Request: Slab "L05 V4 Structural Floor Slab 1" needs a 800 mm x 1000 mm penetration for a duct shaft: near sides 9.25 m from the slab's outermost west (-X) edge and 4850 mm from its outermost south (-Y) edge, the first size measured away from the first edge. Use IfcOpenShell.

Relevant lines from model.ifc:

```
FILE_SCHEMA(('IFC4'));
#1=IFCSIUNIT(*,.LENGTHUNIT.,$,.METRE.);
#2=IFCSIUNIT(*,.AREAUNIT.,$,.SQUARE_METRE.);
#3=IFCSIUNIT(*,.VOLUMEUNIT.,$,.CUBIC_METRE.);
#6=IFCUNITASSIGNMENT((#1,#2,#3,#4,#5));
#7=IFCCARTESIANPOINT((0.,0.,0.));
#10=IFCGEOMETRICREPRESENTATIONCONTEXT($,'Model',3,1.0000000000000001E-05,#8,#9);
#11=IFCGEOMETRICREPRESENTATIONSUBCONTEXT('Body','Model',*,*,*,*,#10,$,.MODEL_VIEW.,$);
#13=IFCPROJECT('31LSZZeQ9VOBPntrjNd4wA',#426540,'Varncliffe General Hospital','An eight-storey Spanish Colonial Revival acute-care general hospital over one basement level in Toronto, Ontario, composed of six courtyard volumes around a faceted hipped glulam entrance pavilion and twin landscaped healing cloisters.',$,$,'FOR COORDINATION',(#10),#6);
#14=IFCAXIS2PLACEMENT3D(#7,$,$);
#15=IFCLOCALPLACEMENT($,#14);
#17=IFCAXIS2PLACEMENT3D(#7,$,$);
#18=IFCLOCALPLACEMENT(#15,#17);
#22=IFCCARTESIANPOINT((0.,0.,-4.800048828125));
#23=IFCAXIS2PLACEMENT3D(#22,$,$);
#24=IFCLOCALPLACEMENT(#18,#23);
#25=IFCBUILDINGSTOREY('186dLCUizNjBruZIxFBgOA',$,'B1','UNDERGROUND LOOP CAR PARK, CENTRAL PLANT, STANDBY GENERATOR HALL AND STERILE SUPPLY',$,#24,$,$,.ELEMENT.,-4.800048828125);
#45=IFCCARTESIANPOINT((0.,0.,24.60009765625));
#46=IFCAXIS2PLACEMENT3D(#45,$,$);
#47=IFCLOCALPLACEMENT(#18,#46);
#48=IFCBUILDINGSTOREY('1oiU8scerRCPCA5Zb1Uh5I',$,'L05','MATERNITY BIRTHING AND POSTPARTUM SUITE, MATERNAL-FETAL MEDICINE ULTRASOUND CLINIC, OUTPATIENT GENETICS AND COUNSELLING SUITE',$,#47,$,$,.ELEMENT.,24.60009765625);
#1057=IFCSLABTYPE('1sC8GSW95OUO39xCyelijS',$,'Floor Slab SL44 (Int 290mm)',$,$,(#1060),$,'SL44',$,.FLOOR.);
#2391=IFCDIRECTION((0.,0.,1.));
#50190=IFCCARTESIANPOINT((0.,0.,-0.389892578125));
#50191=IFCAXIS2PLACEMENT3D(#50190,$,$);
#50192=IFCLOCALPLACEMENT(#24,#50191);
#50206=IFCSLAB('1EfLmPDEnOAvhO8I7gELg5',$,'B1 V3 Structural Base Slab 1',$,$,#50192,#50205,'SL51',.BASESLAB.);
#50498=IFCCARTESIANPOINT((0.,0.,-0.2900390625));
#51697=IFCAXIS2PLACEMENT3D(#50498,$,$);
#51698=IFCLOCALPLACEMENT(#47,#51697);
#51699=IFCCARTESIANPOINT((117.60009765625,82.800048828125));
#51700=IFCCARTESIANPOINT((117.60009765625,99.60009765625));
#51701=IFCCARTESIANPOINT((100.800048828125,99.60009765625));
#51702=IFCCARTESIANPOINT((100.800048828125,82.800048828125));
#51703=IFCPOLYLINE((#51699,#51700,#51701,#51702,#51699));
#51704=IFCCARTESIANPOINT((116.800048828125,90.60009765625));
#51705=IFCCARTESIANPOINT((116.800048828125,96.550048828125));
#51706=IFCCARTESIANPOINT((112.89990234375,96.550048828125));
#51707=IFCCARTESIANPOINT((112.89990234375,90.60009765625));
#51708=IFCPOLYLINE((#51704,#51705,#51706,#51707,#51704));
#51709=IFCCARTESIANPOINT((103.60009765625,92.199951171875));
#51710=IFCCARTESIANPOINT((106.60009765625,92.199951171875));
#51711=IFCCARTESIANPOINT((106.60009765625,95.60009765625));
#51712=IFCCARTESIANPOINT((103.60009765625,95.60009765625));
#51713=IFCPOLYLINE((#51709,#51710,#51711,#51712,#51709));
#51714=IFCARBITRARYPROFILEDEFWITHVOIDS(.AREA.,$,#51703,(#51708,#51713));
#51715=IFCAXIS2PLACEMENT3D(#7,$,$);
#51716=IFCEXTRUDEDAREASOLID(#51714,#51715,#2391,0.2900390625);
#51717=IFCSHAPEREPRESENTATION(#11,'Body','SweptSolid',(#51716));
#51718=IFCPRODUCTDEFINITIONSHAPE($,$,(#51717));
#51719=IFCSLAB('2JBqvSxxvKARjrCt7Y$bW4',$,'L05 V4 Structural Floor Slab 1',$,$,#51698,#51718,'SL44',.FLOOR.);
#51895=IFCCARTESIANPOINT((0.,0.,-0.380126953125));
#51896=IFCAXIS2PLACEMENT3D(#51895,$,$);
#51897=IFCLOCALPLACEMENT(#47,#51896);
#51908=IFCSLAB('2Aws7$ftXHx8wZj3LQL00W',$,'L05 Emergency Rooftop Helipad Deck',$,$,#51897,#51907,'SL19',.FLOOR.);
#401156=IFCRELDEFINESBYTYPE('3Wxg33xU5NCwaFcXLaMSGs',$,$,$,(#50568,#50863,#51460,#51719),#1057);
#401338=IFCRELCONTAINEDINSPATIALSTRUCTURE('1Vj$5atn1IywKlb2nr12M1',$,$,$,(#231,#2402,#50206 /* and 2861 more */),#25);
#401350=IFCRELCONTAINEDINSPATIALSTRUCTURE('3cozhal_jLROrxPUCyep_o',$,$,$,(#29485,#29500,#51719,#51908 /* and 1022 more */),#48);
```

```python
import numpy as np
import ifcopenshell
import ifcopenshell.api.feature
import ifcopenshell.api.geometry
import ifcopenshell.api.root
import ifcopenshell.geom
import ifcopenshell.util.placement
import ifcopenshell.util.representation
import ifcopenshell.util.shape
import ifcopenshell.util.unit

model = ifcopenshell.open("model.ifc")
unit_scale = ifcopenshell.util.unit.calculate_unit_scale(model)
settings = ifcopenshell.geom.settings()


def volume(element):
    """Net volume in cubic metres, openings subtracted."""
    shape = ifcopenshell.geom.create_shape(settings, element)
    return ifcopenshell.util.shape.get_volume(shape.geometry)


slab = model.by_guid("2JBqvSxxvKARjrCt7Y$bW4")
before = volume(slab)

# Extent in the slab's own axes, in metres. The edges named are its -X and -Y sides.
slab_shape = ifcopenshell.geom.create_shape(settings, slab)
vertices = ifcopenshell.util.shape.get_vertices(slab_shape.geometry)
x_min, y_min, bottom = vertices.min(axis=0)
top = vertices[:, 2].max()

opening = ifcopenshell.api.root.create_entity(model, ifc_class="IfcOpeningElement", name="Duct shaft opening", predefined_type="OPENING")
context = ifcopenshell.util.representation.get_context(model, "Model", "Body", "MODEL_VIEW")
width, depth = 0.8, 1
outline = [(0.0, 0.0), (width, 0.0), (width, depth), (0.0, depth), (0.0, 0.0)]
# Overshoot both faces by 50 mm so the cut is clean.
shape = ifcopenshell.api.geometry.add_slab_representation(
    model, context=context, depth=top - bottom + 0.1, polyline=outline
)
ifcopenshell.api.geometry.assign_representation(model, product=opening, representation=shape)

matrix = ifcopenshell.util.placement.get_local_placement(slab.ObjectPlacement)
matrix[:, 3] = matrix @ np.append(np.array([x_min + 9.25, y_min + 4.85, bottom - 0.05]) / unit_scale, 1.0)
ifcopenshell.api.geometry.edit_object_placement(model, product=opening, matrix=matrix, is_si=False)
ifcopenshell.api.feature.add_feature(model, feature=opening, element=slab)

after = volume(slab)

print(f"slab volume {before:.3f} -> {after:.3f} m3")

model.write("model_rev.ifc")
```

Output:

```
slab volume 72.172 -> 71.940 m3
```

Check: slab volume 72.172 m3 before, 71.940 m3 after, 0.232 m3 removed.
